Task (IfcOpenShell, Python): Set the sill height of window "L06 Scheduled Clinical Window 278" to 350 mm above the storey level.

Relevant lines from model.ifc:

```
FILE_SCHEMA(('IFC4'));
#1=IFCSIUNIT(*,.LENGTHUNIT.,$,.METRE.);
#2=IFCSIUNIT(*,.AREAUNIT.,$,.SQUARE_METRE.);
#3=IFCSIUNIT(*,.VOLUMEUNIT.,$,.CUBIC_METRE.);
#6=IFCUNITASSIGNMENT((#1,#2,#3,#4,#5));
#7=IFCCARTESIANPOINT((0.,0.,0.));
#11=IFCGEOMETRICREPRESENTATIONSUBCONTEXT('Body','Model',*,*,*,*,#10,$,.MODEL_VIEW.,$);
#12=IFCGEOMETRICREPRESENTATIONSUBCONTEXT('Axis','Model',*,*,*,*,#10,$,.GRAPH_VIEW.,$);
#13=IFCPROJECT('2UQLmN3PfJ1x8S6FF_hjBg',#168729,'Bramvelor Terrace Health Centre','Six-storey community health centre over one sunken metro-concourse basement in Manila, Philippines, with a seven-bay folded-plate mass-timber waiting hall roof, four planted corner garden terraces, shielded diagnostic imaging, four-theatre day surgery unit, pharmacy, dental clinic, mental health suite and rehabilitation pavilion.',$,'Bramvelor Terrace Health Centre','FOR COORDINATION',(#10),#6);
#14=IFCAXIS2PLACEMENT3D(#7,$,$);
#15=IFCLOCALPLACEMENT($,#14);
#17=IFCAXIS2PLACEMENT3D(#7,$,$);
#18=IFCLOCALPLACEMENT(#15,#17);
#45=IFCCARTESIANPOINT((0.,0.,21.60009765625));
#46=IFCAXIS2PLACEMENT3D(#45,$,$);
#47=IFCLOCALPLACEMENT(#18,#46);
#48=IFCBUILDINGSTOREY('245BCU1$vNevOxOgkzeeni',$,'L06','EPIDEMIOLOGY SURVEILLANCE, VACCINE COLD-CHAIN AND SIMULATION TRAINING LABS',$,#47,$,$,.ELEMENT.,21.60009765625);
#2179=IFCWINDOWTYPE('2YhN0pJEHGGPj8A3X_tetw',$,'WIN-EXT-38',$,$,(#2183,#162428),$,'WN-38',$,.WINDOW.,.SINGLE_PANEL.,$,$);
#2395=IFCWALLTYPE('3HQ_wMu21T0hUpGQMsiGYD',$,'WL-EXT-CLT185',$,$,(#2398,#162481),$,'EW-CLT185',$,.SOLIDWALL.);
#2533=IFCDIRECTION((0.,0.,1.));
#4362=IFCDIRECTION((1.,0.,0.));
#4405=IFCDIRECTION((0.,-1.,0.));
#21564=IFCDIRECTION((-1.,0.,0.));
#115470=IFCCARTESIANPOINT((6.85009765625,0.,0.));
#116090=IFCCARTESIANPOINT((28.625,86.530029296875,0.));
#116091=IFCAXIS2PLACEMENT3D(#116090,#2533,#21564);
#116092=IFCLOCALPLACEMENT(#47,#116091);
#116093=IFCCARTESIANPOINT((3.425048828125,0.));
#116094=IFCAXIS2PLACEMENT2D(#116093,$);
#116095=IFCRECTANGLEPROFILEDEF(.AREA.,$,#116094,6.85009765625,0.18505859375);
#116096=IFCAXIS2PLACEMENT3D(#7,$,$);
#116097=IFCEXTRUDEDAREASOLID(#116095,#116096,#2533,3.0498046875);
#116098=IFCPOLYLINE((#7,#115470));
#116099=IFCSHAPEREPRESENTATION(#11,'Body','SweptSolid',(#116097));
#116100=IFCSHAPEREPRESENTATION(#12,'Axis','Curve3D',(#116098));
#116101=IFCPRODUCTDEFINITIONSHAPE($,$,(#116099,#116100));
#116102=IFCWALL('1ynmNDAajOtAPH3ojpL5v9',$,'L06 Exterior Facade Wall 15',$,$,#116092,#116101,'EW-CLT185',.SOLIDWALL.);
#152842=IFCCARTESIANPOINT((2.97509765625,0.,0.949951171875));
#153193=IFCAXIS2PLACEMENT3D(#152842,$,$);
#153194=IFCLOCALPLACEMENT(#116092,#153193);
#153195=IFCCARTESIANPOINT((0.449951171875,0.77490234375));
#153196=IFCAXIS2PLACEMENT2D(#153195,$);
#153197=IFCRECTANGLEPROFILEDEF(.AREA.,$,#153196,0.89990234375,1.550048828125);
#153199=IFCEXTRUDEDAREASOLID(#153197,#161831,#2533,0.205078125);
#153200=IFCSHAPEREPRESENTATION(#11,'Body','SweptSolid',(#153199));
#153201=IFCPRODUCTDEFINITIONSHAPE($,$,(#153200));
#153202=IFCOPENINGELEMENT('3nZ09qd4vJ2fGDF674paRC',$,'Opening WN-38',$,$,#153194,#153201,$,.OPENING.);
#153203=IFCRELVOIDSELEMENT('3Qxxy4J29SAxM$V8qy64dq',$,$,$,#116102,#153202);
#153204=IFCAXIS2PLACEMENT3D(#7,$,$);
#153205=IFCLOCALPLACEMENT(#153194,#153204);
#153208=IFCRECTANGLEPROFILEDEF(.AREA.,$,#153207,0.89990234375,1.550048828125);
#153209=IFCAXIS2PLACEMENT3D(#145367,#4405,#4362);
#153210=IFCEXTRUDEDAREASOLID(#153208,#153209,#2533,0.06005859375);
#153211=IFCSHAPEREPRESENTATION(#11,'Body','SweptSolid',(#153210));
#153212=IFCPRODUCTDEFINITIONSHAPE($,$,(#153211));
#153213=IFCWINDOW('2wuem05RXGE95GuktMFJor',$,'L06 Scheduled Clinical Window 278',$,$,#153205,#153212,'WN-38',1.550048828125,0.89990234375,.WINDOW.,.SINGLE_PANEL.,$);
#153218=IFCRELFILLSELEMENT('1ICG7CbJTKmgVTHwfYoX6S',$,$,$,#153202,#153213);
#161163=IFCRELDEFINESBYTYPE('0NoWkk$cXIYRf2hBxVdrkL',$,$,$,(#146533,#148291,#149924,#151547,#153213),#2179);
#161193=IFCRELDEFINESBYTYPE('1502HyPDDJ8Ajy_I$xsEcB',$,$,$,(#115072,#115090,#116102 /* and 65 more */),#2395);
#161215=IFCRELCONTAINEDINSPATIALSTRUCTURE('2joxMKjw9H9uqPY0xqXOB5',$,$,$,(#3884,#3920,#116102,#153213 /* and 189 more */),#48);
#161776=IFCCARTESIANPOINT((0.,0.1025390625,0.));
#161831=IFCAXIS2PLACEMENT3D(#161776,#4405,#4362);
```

```python
import numpy as np
import ifcopenshell
import ifcopenshell.api.geometry
import ifcopenshell.geom
import ifcopenshell.util.element
import ifcopenshell.util.placement
import ifcopenshell.util.shape
import ifcopenshell.util.unit

model = ifcopenshell.open("model.ifc")
unit_scale = ifcopenshell.util.unit.calculate_unit_scale(model)

window = model.by_id(153213)
opening = window.FillsVoids[0].RelatingOpeningElement
storey = ifcopenshell.util.element.get_container(window, ifc_class="IfcBuildingStorey")
level = ifcopenshell.util.placement.get_local_placement(storey.ObjectPlacement)[2, 3]

# The opening's origin need not be at the sill, so measure its lowest point.
shape = ifcopenshell.geom.create_shape(ifcopenshell.geom.settings(), opening)
bottom = ifcopenshell.util.shape.get_shape_bottom_elevation(shape, shape.geometry) / unit_scale
dz = level + 0.35 - bottom

shift = np.array([0.0, 0.0, dz])
# The window is placed relative to its opening, so it follows when the opening moves.
matrix = ifcopenshell.util.placement.get_local_placement(opening.ObjectPlacement)
matrix[:3, 3] += shift
ifcopenshell.api.geometry.edit_object_placement(
    model, product=opening, matrix=matrix, is_si=False, should_transform_children=True
)

print(f"moved by {dz * unit_scale:+.3f} m")

model.write("model_rev.ifc")
```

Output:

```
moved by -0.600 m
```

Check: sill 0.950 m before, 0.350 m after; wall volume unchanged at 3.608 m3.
